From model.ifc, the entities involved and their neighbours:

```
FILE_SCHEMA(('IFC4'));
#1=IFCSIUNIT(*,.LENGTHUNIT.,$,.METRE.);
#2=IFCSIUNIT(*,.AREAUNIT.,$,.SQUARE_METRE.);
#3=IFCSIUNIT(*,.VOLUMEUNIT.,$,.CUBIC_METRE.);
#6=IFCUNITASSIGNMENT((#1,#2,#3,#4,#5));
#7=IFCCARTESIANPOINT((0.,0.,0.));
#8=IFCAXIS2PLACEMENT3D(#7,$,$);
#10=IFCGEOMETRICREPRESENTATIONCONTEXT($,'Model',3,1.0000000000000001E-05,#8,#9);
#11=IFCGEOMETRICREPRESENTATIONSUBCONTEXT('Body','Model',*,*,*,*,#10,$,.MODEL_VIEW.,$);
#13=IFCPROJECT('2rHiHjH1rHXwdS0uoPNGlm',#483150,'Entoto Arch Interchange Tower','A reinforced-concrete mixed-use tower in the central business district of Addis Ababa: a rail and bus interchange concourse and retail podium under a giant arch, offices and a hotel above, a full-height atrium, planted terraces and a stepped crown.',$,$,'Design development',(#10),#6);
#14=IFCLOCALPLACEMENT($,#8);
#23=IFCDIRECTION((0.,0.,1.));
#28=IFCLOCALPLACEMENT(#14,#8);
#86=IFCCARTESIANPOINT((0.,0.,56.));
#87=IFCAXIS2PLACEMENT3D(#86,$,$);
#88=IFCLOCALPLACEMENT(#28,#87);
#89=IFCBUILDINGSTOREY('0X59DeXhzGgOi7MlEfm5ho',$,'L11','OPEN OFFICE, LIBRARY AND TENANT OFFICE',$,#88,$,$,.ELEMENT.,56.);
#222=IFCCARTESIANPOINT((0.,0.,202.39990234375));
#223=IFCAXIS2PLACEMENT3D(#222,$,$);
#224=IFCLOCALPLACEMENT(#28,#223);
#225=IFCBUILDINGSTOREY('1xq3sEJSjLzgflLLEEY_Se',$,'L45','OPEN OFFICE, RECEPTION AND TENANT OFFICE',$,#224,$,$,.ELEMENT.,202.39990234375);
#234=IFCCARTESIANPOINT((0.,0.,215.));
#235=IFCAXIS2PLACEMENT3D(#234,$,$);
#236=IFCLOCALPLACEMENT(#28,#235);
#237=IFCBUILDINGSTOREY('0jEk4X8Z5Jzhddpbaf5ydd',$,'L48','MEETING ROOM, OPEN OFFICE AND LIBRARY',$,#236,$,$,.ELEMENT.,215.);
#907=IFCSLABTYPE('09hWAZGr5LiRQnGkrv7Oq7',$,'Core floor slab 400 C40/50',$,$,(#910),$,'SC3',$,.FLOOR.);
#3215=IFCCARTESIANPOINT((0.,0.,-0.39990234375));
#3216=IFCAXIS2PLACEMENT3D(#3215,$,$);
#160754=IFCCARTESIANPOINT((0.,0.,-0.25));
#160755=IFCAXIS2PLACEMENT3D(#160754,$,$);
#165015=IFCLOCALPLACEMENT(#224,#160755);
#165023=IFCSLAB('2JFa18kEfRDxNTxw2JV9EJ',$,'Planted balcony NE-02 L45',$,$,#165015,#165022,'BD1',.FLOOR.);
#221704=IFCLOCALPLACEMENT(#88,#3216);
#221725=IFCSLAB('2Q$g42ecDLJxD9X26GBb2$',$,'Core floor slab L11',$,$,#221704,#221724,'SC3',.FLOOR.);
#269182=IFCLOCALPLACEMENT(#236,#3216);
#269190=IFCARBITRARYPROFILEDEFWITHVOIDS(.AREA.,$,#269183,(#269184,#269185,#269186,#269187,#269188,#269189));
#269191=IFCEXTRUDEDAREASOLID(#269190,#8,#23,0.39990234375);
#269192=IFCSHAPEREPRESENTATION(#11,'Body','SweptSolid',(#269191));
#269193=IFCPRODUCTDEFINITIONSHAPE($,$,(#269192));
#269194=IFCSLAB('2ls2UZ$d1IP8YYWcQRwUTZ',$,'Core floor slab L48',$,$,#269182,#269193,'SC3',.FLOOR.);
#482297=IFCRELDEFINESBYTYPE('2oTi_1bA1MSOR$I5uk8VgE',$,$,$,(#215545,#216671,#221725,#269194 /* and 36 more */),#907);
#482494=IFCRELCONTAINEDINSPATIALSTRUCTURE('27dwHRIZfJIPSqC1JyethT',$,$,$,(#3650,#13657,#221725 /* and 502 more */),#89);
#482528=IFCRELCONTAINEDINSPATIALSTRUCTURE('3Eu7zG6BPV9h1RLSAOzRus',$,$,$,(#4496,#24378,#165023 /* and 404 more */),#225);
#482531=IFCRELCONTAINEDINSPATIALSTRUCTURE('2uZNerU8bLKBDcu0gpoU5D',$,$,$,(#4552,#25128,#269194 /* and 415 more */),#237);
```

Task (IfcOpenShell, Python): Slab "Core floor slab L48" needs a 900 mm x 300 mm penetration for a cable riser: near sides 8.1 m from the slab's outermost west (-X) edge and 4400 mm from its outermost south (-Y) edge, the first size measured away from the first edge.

```python
import numpy as np
import ifcopenshell
import ifcopenshell.api.feature
import ifcopenshell.api.geometry
import ifcopenshell.api.root
import ifcopenshell.geom
import ifcopenshell.util.placement
import ifcopenshell.util.representation
import ifcopenshell.util.shape
import ifcopenshell.util.unit

model = ifcopenshell.open("model.ifc")
unit_scale = ifcopenshell.util.unit.calculate_unit_scale(model)
settings = ifcopenshell.geom.settings()


def volume(element):
    """Net volume in cubic metres, openings subtracted."""
    shape = ifcopenshell.geom.create_shape(settings, element)
    return ifcopenshell.util.shape.get_volume(shape.geometry)


slab = model.by_guid("2ls2UZ$d1IP8YYWcQRwUTZ")
before = volume(slab)

# Extent in the slab's own axes, in metres. The edges named are its -X and -Y sides.
slab_shape = ifcopenshell.geom.create_shape(settings, slab)
vertices = ifcopenshell.util.shape.get_vertices(slab_shape.geometry)
x_min, y_min, bottom = vertices.min(axis=0)
top = vertices[:, 2].max()

opening = ifcopenshell.api.root.create_entity(model, ifc_class="IfcOpeningElement", name="Cable riser opening", predefined_type="OPENING")
context = ifcopenshell.util.representation.get_context(model, "Model", "Body", "MODEL_VIEW")
width, depth = 0.9, 0.3
outline = [(0.0, 0.0), (width, 0.0), (width, depth), (0.0, depth), (0.0, 0.0)]
# Overshoot both faces by 50 mm so the cut is clean.
shape = ifcopenshell.api.geometry.add_slab_representation(
    model, context=context, depth=top - bottom + 0.1, polyline=outline
)
ifcopenshell.api.geometry.assign_representation(model, product=opening, representation=shape)

matrix = ifcopenshell.util.placement.get_local_placement(slab.ObjectPlacement)
matrix[:, 3] = matrix @ np.append(np.array([x_min + 8.1, y_min + 4.4, bottom - 0.05]) / unit_scale, 1.0)
ifcopenshell.api.geometry.edit_object_placement(model, product=opening, matrix=matrix, is_si=False)
ifcopenshell.api.feature.add_feature(model, feature=opening, element=slab)

after = volume(slab)

print(f"slab volume {before:.3f} -> {after:.3f} m3")

model.write("model_rev.ifc")
```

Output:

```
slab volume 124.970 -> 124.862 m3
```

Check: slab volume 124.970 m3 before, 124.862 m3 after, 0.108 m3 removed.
